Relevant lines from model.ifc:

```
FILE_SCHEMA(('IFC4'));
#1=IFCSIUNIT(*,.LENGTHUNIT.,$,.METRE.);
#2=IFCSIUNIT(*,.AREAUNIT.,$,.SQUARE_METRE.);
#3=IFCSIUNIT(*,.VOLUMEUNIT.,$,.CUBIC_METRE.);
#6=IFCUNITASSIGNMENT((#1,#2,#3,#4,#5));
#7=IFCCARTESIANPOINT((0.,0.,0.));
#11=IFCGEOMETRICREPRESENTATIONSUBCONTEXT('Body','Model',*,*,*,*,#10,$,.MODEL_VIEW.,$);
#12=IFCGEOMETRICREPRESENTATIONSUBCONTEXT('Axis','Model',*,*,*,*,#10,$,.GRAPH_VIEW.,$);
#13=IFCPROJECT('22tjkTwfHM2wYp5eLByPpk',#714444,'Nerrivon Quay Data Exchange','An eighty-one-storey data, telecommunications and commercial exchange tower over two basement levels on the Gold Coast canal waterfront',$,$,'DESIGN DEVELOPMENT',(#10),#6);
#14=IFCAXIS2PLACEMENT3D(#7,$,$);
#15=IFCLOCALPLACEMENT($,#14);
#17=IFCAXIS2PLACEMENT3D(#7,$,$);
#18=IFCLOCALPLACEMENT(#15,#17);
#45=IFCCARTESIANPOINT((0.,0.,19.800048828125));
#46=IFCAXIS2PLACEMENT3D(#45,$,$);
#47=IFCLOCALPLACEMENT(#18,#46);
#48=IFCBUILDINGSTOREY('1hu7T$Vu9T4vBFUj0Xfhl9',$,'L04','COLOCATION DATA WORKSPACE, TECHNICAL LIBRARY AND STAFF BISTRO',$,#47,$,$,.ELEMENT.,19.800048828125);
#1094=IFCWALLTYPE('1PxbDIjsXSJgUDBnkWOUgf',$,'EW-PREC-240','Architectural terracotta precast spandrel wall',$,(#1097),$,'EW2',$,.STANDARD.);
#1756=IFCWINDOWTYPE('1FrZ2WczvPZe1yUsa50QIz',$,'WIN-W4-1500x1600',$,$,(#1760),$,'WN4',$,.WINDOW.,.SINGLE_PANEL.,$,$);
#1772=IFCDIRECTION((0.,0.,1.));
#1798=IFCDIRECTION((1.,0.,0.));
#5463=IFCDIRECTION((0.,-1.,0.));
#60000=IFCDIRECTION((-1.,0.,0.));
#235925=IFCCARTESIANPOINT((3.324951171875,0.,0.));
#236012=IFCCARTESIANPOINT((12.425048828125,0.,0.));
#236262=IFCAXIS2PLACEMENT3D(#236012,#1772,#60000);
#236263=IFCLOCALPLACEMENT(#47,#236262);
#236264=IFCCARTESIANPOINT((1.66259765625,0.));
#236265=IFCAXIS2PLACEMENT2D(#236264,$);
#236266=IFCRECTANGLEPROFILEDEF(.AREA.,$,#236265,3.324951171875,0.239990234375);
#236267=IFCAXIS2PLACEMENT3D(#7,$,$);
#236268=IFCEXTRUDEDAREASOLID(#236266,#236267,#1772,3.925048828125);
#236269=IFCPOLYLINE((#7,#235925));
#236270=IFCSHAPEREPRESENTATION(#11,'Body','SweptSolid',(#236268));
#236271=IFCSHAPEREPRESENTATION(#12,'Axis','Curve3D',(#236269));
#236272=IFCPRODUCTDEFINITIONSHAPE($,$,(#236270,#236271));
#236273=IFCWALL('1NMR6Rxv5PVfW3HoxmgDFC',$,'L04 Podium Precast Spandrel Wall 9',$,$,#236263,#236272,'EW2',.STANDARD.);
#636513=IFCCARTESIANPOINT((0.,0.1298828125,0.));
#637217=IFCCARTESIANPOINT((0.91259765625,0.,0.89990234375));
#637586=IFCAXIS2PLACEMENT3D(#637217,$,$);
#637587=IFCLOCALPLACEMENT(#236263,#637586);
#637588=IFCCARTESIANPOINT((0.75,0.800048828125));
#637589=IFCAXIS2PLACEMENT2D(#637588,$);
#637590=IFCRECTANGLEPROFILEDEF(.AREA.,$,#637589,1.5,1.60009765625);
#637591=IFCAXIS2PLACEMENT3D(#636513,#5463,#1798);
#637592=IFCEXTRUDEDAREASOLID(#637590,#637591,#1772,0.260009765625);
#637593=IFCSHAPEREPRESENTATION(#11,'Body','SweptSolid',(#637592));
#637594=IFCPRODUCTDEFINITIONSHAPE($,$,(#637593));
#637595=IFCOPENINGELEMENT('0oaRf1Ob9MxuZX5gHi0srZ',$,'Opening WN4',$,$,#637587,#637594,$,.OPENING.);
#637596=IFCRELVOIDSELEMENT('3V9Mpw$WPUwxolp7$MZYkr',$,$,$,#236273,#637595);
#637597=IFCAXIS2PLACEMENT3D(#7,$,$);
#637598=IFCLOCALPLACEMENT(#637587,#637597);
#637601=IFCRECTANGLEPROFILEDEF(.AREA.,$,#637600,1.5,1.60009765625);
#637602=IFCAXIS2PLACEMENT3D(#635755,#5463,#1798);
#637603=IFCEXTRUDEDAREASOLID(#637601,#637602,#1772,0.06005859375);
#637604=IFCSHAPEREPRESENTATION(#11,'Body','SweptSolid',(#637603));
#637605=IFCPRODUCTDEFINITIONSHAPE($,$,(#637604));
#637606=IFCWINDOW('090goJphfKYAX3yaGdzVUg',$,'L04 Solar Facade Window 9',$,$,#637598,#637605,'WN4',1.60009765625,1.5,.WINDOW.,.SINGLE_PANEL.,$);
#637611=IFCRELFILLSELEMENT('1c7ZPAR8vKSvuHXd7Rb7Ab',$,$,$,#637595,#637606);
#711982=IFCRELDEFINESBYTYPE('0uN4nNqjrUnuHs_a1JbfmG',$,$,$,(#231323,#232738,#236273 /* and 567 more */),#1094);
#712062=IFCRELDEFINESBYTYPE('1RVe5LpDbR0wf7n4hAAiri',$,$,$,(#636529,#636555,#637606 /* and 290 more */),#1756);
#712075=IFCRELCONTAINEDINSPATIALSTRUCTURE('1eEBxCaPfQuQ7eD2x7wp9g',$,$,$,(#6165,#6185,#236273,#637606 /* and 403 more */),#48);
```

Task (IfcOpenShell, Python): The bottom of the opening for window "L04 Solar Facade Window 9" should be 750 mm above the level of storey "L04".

```python
import numpy as np
import ifcopenshell
import ifcopenshell.api.geometry
import ifcopenshell.geom
import ifcopenshell.util.element
import ifcopenshell.util.placement
import ifcopenshell.util.shape
import ifcopenshell.util.unit

model = ifcopenshell.open("model.ifc")
unit_scale = ifcopenshell.util.unit.calculate_unit_scale(model)

window = model.by_id(637606)
opening = window.FillsVoids[0].RelatingOpeningElement
storey = ifcopenshell.util.element.get_container(window, ifc_class="IfcBuildingStorey")
level = ifcopenshell.util.placement.get_local_placement(storey.ObjectPlacement)[2, 3]

# The opening's origin need not be at the sill, so measure its lowest point.
shape = ifcopenshell.geom.create_shape(ifcopenshell.geom.settings(), opening)
bottom = ifcopenshell.util.shape.get_shape_bottom_elevation(shape, shape.geometry) / unit_scale
dz = level + 0.75 / unit_scale - bottom

shift = np.array([0.0, 0.0, dz])
# The window is placed relative to its opening, so it follows when the opening moves.
matrix = ifcopenshell.util.placement.get_local_placement(opening.ObjectPlacement)
matrix[:3, 3] += shift
ifcopenshell.api.geometry.edit_object_placement(
    model, product=opening, matrix=matrix, is_si=False, should_transform_children=True
)

print(f"moved by {dz * unit_scale:+.3f} m")

model.write("model_edited.ifc")
```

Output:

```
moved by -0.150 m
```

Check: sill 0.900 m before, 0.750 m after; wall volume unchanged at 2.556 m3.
